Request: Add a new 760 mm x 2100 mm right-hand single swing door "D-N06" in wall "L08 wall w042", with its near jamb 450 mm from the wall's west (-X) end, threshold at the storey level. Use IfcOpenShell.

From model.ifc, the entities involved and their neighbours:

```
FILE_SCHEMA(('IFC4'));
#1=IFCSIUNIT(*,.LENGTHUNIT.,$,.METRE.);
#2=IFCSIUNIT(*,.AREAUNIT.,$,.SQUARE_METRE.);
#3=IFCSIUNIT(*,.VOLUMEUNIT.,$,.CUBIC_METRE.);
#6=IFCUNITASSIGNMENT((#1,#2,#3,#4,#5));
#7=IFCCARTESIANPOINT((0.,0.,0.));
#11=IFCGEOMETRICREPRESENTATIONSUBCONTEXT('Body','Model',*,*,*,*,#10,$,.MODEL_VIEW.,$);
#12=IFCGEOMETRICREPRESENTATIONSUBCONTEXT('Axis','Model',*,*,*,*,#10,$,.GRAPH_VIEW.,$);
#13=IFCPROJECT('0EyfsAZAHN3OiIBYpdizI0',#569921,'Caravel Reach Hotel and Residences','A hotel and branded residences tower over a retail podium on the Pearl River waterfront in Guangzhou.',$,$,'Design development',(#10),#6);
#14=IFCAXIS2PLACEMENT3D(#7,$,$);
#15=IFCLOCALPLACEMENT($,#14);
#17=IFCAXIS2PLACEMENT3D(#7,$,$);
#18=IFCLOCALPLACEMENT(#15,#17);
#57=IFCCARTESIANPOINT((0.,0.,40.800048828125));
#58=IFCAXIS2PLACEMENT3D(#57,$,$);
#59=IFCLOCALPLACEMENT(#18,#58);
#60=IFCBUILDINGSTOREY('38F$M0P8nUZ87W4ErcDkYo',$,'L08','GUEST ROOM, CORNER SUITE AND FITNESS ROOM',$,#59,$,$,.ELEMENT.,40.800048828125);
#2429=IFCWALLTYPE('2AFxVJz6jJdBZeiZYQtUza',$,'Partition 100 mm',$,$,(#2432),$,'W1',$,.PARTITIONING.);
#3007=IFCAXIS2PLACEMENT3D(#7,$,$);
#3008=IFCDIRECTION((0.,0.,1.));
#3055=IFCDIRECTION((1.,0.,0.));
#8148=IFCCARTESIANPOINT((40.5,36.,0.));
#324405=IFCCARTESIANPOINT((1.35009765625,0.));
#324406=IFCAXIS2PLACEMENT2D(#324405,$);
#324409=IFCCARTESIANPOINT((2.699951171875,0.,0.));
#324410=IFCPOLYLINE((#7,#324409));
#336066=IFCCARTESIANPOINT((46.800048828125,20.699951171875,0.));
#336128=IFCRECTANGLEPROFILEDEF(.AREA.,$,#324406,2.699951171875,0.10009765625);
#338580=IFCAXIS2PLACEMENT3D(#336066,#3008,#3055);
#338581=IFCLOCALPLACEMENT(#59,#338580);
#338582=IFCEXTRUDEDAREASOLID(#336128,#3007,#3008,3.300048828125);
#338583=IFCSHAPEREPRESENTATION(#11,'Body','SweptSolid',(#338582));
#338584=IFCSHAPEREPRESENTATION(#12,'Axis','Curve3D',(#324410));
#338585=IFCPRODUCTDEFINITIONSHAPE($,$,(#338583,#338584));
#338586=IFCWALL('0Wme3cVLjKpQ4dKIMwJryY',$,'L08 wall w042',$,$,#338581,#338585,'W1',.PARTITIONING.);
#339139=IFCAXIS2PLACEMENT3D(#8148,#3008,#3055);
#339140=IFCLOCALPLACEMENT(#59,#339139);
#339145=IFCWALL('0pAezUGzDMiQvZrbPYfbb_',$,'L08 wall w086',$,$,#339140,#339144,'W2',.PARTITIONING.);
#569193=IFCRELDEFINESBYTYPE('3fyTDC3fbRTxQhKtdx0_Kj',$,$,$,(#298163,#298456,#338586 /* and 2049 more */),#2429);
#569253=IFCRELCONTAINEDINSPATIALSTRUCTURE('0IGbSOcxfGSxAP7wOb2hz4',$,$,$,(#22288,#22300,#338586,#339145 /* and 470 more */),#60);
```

```python
import numpy as np
import ifcopenshell
import ifcopenshell.api.feature
import ifcopenshell.api.geometry
import ifcopenshell.api.root
import ifcopenshell.api.spatial
import ifcopenshell.geom
import ifcopenshell.util.element
import ifcopenshell.util.placement
import ifcopenshell.util.representation
import ifcopenshell.util.shape
import ifcopenshell.util.unit

model = ifcopenshell.open("model.ifc")
unit_scale = ifcopenshell.util.unit.calculate_unit_scale(model)
settings = ifcopenshell.geom.settings()


def volume(element):
    """Net volume in cubic metres, openings subtracted."""
    shape = ifcopenshell.geom.create_shape(settings, element)
    return ifcopenshell.util.shape.get_volume(shape.geometry)


wall = model.by_guid("0Wme3cVLjKpQ4dKIMwJryY")
storey = ifcopenshell.util.element.get_container(wall, ifc_class="IfcBuildingStorey")
context = ifcopenshell.util.representation.get_context(model, "Model", "Body", "MODEL_VIEW")
before = volume(wall)

width, height, from_end, sill = 0.76, 2.1, 0.45, 0.0  # metres

# The wall runs along its own X axis, and the end named is its -X end.
wall_shape = ifcopenshell.geom.create_shape(settings, wall)
x, y, z = ifcopenshell.util.shape.get_vertices(wall_shape.geometry).T
start = x.min() + from_end
face, thickness = float(y.min()), float(y.max() - y.min())
wall_matrix = ifcopenshell.util.placement.get_local_placement(wall.ObjectPlacement)
level = ifcopenshell.util.placement.get_local_placement(storey.ObjectPlacement)[2, 3]


def in_wall(x, y):
    """Placement at x, y metres in the wall's axes, at sill height."""
    matrix = wall_matrix.copy()
    matrix[:, 3] = wall_matrix @ np.array([x / unit_scale, y / unit_scale, 0.0, 1.0])
    matrix[2, 3] = level + sill / unit_scale
    return matrix


# Opening: a box that overshoots both wall faces by 50 mm.
opening = ifcopenshell.api.root.create_entity(model, ifc_class="IfcOpeningElement", predefined_type="OPENING")
box = ifcopenshell.api.geometry.add_wall_representation(
    model, context=context, length=width, height=height, thickness=thickness + 0.1
)
ifcopenshell.api.geometry.assign_representation(model, product=opening, representation=box)
ifcopenshell.api.geometry.edit_object_placement(model, product=opening, matrix=in_wall(start, face - 0.05), is_si=False)
ifcopenshell.api.feature.add_feature(model, feature=opening, element=wall)

door = ifcopenshell.api.root.create_entity(model, ifc_class="IfcDoor", name="D-N06", predefined_type="DOOR")
door.OverallWidth, door.OverallHeight = width / unit_scale, height / unit_scale
door.OperationType = "SINGLE_SWING_RIGHT"
body = ifcopenshell.api.geometry.add_door_representation(
    model,
    context=context,
    overall_width=door.OverallWidth,
    overall_height=door.OverallHeight,
    operation_type="SINGLE_SWING_RIGHT",
    lining_properties={"LiningDepth": thickness / unit_scale, "ThresholdDepth": thickness / unit_scale},
)
ifcopenshell.api.geometry.assign_representation(model, product=door, representation=body)
ifcopenshell.api.spatial.assign_container(model, products=[door], relating_structure=storey)
ifcopenshell.api.feature.add_filling(model, opening=opening, element=door)

# The lining spans the wall, so the door starts at the wall face.
ifcopenshell.api.geometry.edit_object_placement(model, product=door, matrix=in_wall(start, face), is_si=False)

after = volume(wall)

print(f"wall volume {before:.3f} -> {after:.3f} m3")

model.write("model-out.ifc")
```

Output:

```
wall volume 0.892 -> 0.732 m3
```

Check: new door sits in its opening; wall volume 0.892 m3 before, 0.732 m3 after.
